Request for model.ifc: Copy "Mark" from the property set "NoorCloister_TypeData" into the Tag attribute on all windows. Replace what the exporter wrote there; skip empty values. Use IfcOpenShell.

First a look at what the model holds.

```python
import ifcopenshell
import ifcopenshell.util.element

model = ifcopenshell.open("model.ifc")
print(model.schema)
windows = model.by_type("IfcWindow")
print(len(windows), "windows")
for e in windows[:8]:
    source = ifcopenshell.util.element.get_pset(e, "NoorCloister_TypeData", "Mark")
    target = e.Tag
    print(e.id(), repr(source), repr(target), sep=" | ")
```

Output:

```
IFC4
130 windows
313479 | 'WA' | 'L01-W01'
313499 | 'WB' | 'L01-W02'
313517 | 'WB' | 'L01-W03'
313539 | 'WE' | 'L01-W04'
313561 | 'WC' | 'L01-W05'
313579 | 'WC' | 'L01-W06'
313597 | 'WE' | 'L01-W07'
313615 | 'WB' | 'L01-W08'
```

```python
import ifcopenshell
import ifcopenshell.util.element

model = ifcopenshell.open("model.ifc")

count = 0
for e in model.by_type("IfcWindow"):
    value = ifcopenshell.util.element.get_pset(e, "NoorCloister_TypeData", "Mark")
    current = e.Tag
    if not value or not value.strip() or current == value:
        continue
    e.Tag = value
    count += 1

print(count, "windows updated")

model.write("model-out.ifc")
```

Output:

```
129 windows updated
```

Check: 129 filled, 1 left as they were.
